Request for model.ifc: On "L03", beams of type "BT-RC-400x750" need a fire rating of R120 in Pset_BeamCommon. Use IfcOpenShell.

First a look at what the model holds.

```python
import ifcopenshell
import ifcopenshell.util.element

model = ifcopenshell.open("model.ifc")
print(model.schema)
storey = next(s for s in model.by_type("IfcBuildingStorey") if s.Name == "L03")
beams = [e for e in ifcopenshell.util.element.get_decomposition(storey) if e.is_a("IfcBeam")]
seen = {}
for e in beams:
    element_type = ifcopenshell.util.element.get_type(e)
    key = (element_type.Name if element_type != e and element_type else None, ifcopenshell.util.element.get_pset(e, "Pset_BeamCommon", "FireRating"))
    seen[key] = seen.get(key, 0) + 1
for (name, value), count in sorted(seen.items(), key=str):
    print(count, "x", name, "|", value)
```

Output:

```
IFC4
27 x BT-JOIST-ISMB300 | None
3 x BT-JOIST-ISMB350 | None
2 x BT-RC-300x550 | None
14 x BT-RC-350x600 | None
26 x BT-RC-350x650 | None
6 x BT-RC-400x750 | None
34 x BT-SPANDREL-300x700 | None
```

```python
import ifcopenshell
import ifcopenshell.api.pset
import ifcopenshell.util.element

model = ifcopenshell.open("model.ifc")

storey = next(s for s in model.by_type("IfcBuildingStorey") if s.Name == "L03")
beams = [e for e in ifcopenshell.util.element.get_decomposition(storey) if e.is_a("IfcBeam")]

count = 0
for e in beams:
    element_type = ifcopenshell.util.element.get_type(e)
    if element_type in (None, e) or element_type.Name != "BT-RC-400x750":
        continue
    # add_pset returns the element's existing set when there is one.
    pset = ifcopenshell.api.pset.add_pset(model, product=e, name="Pset_BeamCommon")
    ifcopenshell.api.pset.edit_pset(model, pset=pset, properties={"FireRating": "R120"})
    count += 1

print(count, "beams updated")

model.write("model-out.ifc")
```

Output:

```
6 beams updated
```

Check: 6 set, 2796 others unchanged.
